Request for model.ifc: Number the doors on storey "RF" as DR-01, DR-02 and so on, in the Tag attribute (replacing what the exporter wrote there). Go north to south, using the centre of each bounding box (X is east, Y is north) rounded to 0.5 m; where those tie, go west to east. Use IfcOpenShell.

First a look at what the model holds.

```python
import ifcopenshell
import ifcopenshell.util.element
import ifcopenshell.util.placement

model = ifcopenshell.open("model.ifc")
print(model.schema)
storey = next(s for s in model.by_type("IfcBuildingStorey") if s.Name == "RF")
doors = [e for e in ifcopenshell.util.element.get_decomposition(storey) if e.is_a("IfcDoor")]
for e in sorted(doors, key=lambda e: e.id()):
    origin = ifcopenshell.util.placement.get_local_placement(e.ObjectPlacement)[:3, 3]
    print(e.id(), e.Tag, e.Name, origin.round(2) + 0.0, sep=" | ")
```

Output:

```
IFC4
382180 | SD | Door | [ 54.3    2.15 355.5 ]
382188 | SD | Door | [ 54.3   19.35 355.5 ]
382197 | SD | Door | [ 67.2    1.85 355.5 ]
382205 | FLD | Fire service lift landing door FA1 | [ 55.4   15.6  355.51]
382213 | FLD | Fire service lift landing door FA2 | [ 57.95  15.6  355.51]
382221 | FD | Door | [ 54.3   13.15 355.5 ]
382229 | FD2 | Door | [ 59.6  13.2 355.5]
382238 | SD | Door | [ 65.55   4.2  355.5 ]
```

```python
import ifcopenshell
import ifcopenshell.geom
import ifcopenshell.util.element
import ifcopenshell.util.shape

model = ifcopenshell.open("model.ifc")
settings = ifcopenshell.geom.settings()
settings.set("use-world-coords", True)


def centre(element):
    shape = ifcopenshell.geom.create_shape(settings, element)
    return ifcopenshell.util.shape.get_bbox_centroid(shape.geometry)


storey = next(s for s in model.by_type("IfcBuildingStorey") if s.Name == "RF")
doors = [e for e in ifcopenshell.util.element.get_decomposition(storey) if e.is_a("IfcDoor")]

# Insertion points can sit at a corner or the storey origin, so sort by the geometry (in metres).
centres = {e: centre(e) for e in doors}
doors.sort(key=lambda e: (-round(centres[e][1] / 0.5), centres[e][0]))

for i, e in enumerate(doors, start=1):
    number = f"DR-{i:02d}"
    e.Tag = number
    print(e.id(), number)

model.write("model_v2.ifc")
```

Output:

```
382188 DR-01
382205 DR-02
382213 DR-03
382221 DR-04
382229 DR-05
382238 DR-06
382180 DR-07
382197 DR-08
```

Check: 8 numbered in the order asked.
